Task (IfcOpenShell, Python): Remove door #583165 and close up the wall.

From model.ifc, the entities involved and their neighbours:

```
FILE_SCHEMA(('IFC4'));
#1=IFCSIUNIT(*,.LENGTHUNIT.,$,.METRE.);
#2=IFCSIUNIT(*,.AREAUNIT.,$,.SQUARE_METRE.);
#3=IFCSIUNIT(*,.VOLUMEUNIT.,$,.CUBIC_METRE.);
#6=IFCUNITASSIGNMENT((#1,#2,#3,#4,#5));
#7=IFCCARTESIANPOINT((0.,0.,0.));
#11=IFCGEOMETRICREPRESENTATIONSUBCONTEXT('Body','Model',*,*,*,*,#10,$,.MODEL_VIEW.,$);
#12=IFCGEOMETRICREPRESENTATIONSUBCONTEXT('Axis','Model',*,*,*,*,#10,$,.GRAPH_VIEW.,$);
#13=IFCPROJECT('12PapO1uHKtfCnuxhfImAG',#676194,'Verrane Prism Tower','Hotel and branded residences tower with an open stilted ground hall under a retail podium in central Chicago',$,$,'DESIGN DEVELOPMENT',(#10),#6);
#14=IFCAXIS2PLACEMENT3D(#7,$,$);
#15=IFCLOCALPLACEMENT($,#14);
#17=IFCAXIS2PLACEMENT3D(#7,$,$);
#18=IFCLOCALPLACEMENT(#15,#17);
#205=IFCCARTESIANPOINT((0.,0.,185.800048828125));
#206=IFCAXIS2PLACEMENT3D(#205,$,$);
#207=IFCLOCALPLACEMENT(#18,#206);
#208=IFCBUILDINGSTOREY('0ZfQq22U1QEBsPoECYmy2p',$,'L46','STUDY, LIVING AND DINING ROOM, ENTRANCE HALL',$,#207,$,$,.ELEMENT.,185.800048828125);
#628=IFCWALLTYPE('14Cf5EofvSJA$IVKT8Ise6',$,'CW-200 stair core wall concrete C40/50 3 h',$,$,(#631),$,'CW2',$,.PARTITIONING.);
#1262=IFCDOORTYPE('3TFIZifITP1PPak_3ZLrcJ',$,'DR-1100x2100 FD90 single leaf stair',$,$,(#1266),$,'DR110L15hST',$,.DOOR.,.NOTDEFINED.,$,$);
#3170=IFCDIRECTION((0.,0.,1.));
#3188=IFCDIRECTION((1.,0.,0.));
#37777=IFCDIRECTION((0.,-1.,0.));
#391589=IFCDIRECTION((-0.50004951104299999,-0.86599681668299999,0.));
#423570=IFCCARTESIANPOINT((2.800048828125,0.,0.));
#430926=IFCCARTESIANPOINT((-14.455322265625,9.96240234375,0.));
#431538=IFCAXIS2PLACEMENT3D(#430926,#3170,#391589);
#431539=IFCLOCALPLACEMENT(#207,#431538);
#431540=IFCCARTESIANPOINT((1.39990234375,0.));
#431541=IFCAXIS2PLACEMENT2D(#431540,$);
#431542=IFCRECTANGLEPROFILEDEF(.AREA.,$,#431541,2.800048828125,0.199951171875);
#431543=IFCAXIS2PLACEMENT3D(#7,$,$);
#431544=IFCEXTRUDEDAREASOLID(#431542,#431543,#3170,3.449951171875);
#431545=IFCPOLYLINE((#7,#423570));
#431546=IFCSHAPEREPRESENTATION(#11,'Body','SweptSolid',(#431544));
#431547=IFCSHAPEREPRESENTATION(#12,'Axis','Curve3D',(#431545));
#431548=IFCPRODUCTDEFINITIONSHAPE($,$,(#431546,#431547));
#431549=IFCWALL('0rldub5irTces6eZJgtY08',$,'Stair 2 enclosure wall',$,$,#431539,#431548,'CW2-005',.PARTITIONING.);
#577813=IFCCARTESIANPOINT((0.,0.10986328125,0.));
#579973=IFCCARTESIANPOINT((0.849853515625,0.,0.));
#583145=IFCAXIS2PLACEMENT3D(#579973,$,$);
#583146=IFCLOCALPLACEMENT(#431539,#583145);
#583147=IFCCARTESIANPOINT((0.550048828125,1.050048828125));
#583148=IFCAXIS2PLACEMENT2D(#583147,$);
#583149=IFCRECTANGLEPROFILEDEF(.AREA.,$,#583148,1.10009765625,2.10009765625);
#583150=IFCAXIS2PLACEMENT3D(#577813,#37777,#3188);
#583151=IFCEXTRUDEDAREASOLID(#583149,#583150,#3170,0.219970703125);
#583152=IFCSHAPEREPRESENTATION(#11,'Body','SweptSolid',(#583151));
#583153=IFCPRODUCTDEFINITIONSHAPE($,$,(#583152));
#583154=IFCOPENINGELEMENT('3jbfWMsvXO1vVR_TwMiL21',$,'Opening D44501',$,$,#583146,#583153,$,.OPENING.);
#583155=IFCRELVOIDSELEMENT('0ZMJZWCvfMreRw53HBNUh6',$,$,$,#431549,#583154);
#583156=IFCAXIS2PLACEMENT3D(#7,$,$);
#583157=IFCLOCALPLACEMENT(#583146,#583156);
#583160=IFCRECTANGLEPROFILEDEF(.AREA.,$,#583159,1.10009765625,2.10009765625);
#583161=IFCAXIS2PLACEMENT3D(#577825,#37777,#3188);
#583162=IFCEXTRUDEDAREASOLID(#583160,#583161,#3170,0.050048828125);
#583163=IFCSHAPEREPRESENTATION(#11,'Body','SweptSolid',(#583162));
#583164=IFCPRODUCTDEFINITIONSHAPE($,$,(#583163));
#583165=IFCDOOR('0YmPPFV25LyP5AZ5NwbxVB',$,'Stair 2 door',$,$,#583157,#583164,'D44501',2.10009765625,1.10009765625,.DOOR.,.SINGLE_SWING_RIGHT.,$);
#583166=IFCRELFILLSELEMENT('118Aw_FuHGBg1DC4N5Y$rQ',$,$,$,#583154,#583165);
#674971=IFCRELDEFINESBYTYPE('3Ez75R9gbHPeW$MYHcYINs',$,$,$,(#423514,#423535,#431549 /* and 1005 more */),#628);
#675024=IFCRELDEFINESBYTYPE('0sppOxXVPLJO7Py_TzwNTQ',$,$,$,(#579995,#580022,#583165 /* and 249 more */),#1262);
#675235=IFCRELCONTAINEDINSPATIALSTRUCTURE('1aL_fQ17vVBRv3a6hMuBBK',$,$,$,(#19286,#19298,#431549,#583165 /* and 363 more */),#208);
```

```python
import ifcopenshell
import ifcopenshell.api.feature
import ifcopenshell.api.root
import ifcopenshell.geom
import ifcopenshell.util.shape

model = ifcopenshell.open("model.ifc")
settings = ifcopenshell.geom.settings()


def volume(element):
    """Net volume in cubic metres, openings subtracted."""
    shape = ifcopenshell.geom.create_shape(settings, element)
    return ifcopenshell.util.shape.get_volume(shape.geometry)


door = model.by_id(583165)
opening = door.FillsVoids[0].RelatingOpeningElement
wall = opening.VoidsElements[0].RelatingBuildingElement
before = volume(wall)

ifcopenshell.api.root.remove_product(model, product=door)
ifcopenshell.api.feature.remove_feature(model, feature=opening)

after = volume(wall)

print(f"wall volume {before:.3f} -> {after:.3f} m3")

model.write("model-out.ifc")
```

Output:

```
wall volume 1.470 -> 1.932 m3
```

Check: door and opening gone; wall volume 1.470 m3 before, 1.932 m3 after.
